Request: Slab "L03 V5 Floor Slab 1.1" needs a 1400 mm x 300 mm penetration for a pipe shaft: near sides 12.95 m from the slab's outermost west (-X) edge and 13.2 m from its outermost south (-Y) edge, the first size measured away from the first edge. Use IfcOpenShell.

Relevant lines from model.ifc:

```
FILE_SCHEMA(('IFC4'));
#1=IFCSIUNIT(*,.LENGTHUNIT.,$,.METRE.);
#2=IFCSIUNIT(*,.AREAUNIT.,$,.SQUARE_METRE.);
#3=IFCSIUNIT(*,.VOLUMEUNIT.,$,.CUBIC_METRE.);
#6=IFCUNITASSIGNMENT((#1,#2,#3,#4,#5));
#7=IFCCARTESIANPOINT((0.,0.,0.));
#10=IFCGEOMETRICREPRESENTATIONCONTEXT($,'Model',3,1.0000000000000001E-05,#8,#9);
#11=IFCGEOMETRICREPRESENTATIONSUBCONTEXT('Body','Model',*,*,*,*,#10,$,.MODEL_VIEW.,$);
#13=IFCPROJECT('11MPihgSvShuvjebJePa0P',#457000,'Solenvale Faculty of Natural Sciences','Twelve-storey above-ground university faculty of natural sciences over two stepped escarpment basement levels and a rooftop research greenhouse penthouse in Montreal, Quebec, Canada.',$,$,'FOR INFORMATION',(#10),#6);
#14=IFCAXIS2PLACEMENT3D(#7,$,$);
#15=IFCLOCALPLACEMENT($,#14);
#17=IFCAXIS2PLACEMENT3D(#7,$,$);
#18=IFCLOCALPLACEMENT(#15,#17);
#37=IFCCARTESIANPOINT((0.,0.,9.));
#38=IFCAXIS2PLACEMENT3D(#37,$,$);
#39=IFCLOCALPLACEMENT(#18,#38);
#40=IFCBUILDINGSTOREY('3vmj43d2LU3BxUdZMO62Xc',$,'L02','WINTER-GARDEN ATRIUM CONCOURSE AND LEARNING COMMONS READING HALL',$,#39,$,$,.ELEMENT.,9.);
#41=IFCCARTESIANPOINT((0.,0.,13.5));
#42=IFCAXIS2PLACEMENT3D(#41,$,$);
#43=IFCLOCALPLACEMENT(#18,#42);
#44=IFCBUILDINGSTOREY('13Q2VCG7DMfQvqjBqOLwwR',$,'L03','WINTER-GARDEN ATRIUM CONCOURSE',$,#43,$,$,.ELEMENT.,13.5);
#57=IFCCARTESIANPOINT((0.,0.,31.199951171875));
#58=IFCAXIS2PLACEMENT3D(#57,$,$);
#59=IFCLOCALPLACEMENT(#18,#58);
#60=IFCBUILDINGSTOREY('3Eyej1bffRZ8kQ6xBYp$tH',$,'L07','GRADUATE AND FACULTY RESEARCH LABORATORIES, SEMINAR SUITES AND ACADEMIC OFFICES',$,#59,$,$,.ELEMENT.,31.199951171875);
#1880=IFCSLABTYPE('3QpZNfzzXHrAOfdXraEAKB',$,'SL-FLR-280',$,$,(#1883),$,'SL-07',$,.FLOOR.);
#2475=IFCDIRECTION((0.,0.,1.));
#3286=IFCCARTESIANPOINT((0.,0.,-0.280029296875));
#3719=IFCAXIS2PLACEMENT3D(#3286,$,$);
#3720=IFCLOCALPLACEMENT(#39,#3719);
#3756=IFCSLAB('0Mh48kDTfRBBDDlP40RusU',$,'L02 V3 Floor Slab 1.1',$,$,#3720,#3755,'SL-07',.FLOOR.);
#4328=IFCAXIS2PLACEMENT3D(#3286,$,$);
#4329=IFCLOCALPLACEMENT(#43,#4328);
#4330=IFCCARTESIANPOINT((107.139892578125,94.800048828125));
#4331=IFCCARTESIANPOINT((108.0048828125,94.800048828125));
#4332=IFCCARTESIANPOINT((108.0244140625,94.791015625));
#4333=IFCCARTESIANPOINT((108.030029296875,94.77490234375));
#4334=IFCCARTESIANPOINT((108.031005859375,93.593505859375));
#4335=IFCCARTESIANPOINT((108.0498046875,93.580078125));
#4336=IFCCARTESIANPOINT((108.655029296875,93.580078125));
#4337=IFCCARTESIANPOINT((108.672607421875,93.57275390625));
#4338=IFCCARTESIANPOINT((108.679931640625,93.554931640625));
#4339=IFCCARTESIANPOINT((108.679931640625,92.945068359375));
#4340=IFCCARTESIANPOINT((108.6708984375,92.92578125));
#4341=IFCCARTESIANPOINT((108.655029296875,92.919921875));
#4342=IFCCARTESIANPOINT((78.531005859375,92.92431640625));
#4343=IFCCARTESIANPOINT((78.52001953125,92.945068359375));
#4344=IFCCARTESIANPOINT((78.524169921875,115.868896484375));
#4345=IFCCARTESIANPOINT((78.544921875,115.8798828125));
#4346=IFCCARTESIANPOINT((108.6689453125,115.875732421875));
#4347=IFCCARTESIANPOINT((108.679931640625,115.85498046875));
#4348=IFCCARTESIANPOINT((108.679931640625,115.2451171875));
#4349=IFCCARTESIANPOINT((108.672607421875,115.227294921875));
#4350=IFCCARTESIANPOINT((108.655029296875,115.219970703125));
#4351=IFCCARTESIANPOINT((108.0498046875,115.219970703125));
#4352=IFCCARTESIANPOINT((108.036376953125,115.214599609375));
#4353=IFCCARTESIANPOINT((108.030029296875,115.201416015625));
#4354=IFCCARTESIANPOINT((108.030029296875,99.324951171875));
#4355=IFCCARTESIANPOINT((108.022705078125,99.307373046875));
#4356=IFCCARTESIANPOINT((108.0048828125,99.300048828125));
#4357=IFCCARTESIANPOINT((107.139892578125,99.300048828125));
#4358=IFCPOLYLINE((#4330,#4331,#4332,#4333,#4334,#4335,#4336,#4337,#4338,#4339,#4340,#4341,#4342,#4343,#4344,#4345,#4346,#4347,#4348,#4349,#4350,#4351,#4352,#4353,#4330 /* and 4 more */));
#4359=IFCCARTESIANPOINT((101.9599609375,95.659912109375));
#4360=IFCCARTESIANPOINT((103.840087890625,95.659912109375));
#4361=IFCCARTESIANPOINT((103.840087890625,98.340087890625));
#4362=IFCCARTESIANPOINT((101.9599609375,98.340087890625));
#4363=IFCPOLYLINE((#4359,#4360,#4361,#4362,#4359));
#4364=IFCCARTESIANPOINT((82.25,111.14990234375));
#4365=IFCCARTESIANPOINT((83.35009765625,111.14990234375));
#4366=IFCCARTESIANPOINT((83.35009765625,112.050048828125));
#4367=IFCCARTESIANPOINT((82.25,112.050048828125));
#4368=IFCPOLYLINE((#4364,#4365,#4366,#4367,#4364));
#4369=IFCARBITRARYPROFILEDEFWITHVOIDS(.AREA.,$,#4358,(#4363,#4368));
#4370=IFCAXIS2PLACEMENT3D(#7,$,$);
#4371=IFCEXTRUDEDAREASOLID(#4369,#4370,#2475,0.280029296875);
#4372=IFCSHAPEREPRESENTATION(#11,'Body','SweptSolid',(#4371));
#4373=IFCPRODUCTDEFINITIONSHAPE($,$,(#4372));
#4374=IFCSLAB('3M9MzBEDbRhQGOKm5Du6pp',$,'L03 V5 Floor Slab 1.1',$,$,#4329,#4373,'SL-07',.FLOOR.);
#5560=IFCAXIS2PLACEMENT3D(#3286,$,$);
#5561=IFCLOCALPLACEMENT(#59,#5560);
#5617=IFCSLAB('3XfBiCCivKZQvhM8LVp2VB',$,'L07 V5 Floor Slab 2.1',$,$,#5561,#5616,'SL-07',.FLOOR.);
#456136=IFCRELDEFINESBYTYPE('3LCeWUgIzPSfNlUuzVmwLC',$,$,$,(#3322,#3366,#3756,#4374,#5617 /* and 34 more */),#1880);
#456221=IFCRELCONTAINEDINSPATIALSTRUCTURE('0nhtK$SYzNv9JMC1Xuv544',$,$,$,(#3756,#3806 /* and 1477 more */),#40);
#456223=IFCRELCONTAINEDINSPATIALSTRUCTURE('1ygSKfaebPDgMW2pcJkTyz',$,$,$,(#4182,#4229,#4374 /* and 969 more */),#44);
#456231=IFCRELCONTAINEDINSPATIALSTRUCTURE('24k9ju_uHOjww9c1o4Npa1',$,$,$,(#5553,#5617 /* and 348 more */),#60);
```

```python
import numpy as np
import ifcopenshell
import ifcopenshell.api.feature
import ifcopenshell.api.geometry
import ifcopenshell.api.root
import ifcopenshell.geom
import ifcopenshell.util.placement
import ifcopenshell.util.representation
import ifcopenshell.util.shape
import ifcopenshell.util.unit

model = ifcopenshell.open("model.ifc")
unit_scale = ifcopenshell.util.unit.calculate_unit_scale(model)
settings = ifcopenshell.geom.settings()


def volume(element):
    """Net volume in cubic metres, openings subtracted."""
    shape = ifcopenshell.geom.create_shape(settings, element)
    return ifcopenshell.util.shape.get_volume(shape.geometry)


slab = model.by_guid("3M9MzBEDbRhQGOKm5Du6pp")
before = volume(slab)

# Extent in the slab's own axes, in metres. The edges named are its -X and -Y sides.
slab_shape = ifcopenshell.geom.create_shape(settings, slab)
vertices = ifcopenshell.util.shape.get_vertices(slab_shape.geometry)
x_min, y_min, bottom = vertices.min(axis=0)
top = vertices[:, 2].max()

opening = ifcopenshell.api.root.create_entity(model, ifc_class="IfcOpeningElement", name="Pipe shaft opening", predefined_type="OPENING")
context = ifcopenshell.util.representation.get_context(model, "Model", "Body", "MODEL_VIEW")
width, depth = 1.4, 0.3
outline = [(0.0, 0.0), (width, 0.0), (width, depth), (0.0, depth), (0.0, 0.0)]
# Overshoot both faces by 50 mm so the cut is clean.
shape = ifcopenshell.api.geometry.add_slab_representation(
    model, context=context, depth=top - bottom + 0.1, polyline=outline
)
ifcopenshell.api.geometry.assign_representation(model, product=opening, representation=shape)

matrix = ifcopenshell.util.placement.get_local_placement(slab.ObjectPlacement)
matrix[:, 3] = matrix @ np.append(np.array([x_min + 12.95, y_min + 13.2, bottom - 0.05]) / unit_scale, 1.0)
ifcopenshell.api.geometry.edit_object_placement(model, product=opening, matrix=matrix, is_si=False)
ifcopenshell.api.feature.add_feature(model, feature=opening, element=slab)

after = volume(slab)

print(f"slab volume {before:.3f} -> {after:.3f} m3")

model.write("model-out.ifc")
```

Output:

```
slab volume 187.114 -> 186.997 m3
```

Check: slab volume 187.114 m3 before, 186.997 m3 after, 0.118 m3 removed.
